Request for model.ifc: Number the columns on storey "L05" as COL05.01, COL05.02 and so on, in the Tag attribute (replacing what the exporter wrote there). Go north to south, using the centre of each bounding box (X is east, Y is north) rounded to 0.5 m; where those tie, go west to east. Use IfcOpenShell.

First a look at what the model holds.

```python
import ifcopenshell
import ifcopenshell.util.element
import ifcopenshell.util.placement

model = ifcopenshell.open("model.ifc")
print(model.schema)
storey = next(s for s in model.by_type("IfcBuildingStorey") if s.Name == "L05")
columns = [e for e in ifcopenshell.util.element.get_decomposition(storey) if e.is_a("IfcColumn")]
for e in sorted(columns, key=lambda e: e.id()):
    origin = ifcopenshell.util.placement.get_local_placement(e.ObjectPlacement)[:3, 3]
    print(e.id(), e.Tag, e.Name, origin.round(2) + 0.0, sep=" | ")
```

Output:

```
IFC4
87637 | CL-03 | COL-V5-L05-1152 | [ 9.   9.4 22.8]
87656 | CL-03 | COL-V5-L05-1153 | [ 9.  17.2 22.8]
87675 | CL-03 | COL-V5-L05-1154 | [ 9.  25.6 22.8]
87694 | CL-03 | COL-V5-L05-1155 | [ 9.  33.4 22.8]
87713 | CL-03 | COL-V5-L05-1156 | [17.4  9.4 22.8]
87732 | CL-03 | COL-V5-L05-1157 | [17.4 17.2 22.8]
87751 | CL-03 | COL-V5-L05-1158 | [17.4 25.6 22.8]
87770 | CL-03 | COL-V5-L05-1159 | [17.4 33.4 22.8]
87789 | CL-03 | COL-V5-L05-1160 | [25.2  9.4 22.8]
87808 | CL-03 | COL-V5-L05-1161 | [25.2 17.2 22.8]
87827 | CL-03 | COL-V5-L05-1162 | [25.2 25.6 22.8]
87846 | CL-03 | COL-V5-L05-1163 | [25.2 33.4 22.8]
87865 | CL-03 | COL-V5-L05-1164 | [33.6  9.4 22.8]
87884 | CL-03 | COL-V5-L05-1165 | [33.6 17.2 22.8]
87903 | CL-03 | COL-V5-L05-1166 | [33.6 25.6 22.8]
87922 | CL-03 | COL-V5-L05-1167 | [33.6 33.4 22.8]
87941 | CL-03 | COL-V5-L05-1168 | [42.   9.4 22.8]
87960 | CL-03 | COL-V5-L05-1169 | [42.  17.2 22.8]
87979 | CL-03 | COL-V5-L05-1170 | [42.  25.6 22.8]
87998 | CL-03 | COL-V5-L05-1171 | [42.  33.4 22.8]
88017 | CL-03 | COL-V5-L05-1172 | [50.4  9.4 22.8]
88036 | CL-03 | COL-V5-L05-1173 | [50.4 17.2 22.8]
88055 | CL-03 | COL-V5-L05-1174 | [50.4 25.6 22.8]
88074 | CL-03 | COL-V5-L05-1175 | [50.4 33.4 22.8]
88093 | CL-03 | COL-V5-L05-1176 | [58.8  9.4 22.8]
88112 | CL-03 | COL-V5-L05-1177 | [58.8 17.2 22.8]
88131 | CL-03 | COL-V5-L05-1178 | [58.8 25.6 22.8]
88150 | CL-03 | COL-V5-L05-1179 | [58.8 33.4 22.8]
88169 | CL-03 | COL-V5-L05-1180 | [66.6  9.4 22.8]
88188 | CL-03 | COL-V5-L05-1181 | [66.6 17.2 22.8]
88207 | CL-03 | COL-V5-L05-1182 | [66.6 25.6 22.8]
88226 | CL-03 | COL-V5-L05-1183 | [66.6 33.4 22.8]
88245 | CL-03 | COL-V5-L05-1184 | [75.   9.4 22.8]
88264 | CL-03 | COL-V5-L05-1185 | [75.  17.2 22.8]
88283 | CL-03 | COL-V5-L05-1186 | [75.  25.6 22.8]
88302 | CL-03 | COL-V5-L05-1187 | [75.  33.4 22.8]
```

```python
import ifcopenshell
import ifcopenshell.geom
import ifcopenshell.util.element
import ifcopenshell.util.shape

model = ifcopenshell.open("model.ifc")
settings = ifcopenshell.geom.settings()
settings.set("use-world-coords", True)


def centre(element):
    shape = ifcopenshell.geom.create_shape(settings, element)
    return ifcopenshell.util.shape.get_bbox_centroid(shape.geometry)


storey = next(s for s in model.by_type("IfcBuildingStorey") if s.Name == "L05")
columns = [e for e in ifcopenshell.util.element.get_decomposition(storey) if e.is_a("IfcColumn")]

# Insertion points can sit at a corner or the storey origin, so sort by the geometry (in metres).
centres = {e: centre(e) for e in columns}
columns.sort(key=lambda e: (-round(centres[e][1] / 0.5), centres[e][0]))

for i, e in enumerate(columns, start=1):
    number = f"COL05.{i:02d}"
    e.Tag = number
    print(e.id(), number)

model.write("model_edited.ifc")
```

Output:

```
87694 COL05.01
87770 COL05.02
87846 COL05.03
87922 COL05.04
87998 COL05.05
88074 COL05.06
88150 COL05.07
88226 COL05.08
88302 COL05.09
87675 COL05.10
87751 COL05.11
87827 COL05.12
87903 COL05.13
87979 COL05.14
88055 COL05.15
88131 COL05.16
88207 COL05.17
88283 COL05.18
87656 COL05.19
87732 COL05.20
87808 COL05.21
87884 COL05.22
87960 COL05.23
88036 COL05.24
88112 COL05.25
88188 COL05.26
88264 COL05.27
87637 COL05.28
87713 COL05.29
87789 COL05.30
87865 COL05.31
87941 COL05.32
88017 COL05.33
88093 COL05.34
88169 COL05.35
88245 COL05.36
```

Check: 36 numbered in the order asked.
